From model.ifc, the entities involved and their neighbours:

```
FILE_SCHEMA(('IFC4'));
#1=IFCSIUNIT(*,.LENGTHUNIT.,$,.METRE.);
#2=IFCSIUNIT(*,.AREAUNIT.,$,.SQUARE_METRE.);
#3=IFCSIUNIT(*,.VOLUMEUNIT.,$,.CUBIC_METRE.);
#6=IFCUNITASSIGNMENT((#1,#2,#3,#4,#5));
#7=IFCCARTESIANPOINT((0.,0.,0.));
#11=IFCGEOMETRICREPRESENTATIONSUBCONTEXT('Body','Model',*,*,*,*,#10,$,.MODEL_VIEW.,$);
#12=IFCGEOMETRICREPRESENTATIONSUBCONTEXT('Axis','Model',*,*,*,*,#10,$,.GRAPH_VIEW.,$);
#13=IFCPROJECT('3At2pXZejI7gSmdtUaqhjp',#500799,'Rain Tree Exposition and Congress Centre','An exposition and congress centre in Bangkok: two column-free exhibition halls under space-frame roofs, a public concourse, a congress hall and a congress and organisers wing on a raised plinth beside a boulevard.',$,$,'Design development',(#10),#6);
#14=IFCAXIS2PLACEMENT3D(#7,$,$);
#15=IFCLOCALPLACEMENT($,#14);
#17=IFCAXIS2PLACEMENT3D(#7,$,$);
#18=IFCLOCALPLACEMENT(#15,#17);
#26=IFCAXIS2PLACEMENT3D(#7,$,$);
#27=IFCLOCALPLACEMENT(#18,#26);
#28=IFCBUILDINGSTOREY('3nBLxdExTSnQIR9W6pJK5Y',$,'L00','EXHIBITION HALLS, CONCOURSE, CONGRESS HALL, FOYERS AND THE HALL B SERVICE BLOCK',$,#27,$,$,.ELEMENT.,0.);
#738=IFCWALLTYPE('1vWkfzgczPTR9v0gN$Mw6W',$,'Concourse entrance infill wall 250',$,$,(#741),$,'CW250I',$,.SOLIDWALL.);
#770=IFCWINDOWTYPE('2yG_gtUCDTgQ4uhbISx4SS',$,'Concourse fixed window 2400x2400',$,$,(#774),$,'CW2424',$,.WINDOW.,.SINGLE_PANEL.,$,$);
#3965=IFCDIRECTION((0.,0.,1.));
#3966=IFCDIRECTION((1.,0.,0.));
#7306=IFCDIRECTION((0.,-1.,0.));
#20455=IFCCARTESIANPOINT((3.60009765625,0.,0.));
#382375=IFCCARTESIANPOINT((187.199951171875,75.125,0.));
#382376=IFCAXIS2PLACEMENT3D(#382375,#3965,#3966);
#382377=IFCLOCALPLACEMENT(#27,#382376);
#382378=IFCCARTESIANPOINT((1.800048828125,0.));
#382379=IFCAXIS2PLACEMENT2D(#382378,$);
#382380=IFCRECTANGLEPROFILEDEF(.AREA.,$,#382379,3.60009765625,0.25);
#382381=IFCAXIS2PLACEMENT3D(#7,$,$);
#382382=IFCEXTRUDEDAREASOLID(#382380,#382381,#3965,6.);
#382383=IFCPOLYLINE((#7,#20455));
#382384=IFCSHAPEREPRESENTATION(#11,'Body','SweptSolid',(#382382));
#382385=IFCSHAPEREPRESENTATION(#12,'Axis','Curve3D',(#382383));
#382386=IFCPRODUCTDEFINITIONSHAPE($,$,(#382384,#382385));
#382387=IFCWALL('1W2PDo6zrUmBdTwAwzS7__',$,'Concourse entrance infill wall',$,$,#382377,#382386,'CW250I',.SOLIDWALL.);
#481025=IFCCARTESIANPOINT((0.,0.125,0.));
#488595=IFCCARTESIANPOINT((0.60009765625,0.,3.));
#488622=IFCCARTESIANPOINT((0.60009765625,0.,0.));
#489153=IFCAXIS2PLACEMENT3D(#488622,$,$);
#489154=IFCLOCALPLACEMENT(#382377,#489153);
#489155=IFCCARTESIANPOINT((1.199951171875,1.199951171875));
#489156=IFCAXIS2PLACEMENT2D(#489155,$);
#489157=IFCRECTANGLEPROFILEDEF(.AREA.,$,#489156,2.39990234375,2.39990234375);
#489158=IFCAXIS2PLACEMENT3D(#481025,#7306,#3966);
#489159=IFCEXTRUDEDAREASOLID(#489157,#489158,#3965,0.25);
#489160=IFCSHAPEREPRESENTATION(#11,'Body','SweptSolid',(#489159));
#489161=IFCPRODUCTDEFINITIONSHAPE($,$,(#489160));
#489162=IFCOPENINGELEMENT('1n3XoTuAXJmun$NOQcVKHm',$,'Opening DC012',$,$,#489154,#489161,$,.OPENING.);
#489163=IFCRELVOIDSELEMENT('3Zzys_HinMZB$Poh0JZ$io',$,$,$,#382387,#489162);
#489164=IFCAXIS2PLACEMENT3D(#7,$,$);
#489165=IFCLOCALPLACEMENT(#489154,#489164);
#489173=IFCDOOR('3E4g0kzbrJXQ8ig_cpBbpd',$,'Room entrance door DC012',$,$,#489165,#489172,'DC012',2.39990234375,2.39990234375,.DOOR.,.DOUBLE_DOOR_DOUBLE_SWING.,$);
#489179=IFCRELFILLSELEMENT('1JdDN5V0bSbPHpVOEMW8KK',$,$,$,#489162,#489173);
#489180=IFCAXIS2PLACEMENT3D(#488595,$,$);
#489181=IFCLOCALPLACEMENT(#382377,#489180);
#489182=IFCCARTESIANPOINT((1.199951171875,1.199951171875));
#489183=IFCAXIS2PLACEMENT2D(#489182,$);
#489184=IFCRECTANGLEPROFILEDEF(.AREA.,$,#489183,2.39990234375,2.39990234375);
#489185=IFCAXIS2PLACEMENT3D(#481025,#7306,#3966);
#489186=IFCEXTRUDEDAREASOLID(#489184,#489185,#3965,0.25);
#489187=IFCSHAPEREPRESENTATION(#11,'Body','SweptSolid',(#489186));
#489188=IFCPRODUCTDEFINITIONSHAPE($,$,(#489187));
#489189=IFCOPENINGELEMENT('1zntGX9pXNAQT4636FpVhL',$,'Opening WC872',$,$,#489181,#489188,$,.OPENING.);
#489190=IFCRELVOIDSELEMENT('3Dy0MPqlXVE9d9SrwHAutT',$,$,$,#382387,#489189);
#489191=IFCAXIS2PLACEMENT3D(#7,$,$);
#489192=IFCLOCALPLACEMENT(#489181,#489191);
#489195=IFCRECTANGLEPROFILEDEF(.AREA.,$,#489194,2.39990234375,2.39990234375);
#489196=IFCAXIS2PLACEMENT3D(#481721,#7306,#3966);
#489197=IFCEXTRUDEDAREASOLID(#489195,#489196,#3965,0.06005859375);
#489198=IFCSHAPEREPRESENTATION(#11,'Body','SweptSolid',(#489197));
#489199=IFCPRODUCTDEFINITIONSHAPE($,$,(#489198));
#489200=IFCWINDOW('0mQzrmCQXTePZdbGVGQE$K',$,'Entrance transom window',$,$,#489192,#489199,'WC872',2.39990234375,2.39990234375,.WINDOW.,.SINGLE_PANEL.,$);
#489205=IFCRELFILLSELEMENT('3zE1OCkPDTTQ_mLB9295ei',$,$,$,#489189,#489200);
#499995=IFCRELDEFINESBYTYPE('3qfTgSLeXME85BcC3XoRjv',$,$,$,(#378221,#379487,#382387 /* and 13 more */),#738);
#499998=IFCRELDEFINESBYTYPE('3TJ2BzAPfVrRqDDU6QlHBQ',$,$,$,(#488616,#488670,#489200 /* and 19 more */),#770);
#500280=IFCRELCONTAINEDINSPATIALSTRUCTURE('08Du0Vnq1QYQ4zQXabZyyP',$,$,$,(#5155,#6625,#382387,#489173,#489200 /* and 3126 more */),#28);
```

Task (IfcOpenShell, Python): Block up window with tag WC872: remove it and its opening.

```python
import ifcopenshell
import ifcopenshell.api.feature
import ifcopenshell.api.root
import ifcopenshell.geom
import ifcopenshell.util.shape

model = ifcopenshell.open("model.ifc")
settings = ifcopenshell.geom.settings()


def volume(element):
    """Net volume in cubic metres, openings subtracted."""
    shape = ifcopenshell.geom.create_shape(settings, element)
    return ifcopenshell.util.shape.get_volume(shape.geometry)


window = model.by_id(489200)
opening = window.FillsVoids[0].RelatingOpeningElement
wall = opening.VoidsElements[0].RelatingBuildingElement
before = volume(wall)

ifcopenshell.api.root.remove_product(model, product=window)
ifcopenshell.api.feature.remove_feature(model, feature=opening)

after = volume(wall)

print(f"wall volume {before:.3f} -> {after:.3f} m3")

model.write("model_updated.ifc")
```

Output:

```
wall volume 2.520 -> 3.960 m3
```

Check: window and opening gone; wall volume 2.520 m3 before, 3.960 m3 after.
